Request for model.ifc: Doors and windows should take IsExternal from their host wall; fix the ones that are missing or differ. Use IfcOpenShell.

First a look at what the model holds.

```python
import ifcopenshell
import ifcopenshell.util.element

model = ifcopenshell.open("model.ifc")
print(model.schema)
seen = {}
for e in model.by_type("IfcDoor") + model.by_type("IfcWindow"):
    if not e.FillsVoids:
        continue
    host = e.FillsVoids[0].RelatingOpeningElement.VoidsElements[0].RelatingBuildingElement
    own = ifcopenshell.util.element.get_pset(e, f"Pset_{e.is_a()[3:].removesuffix('StandardCase')}Common", "IsExternal")
    wall = ifcopenshell.util.element.get_pset(host, "Pset_WallCommon", "IsExternal")
    seen[e.is_a(), own, wall] = seen.get((e.is_a(), own, wall), 0) + 1
for (cls, own, wall), count in sorted(seen.items(), key=str):
    print(count, cls, "IsExternal:", own, "| host wall:", wall)
```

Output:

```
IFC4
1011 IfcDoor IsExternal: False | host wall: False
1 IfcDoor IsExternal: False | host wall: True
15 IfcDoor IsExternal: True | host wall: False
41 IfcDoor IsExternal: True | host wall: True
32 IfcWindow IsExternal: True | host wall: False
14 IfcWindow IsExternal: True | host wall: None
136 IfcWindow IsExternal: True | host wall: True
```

```python
import ifcopenshell
import ifcopenshell.api.pset
import ifcopenshell.util.element

model = ifcopenshell.open("model.ifc")

count = 0
for ifc_class, pset_name in (("IfcDoor", "Pset_DoorCommon"), ("IfcWindow", "Pset_WindowCommon")):
    for e in model.by_type(ifc_class):
        if not e.FillsVoids:
            continue
        host = e.FillsVoids[0].RelatingOpeningElement.VoidsElements[0].RelatingBuildingElement
        external = ifcopenshell.util.element.get_pset(host, "Pset_WallCommon", "IsExternal")
        if external is None or ifcopenshell.util.element.get_pset(e, pset_name, "IsExternal") == external:
            continue
        pset = ifcopenshell.api.pset.add_pset(model, product=e, name=pset_name)
        ifcopenshell.api.pset.edit_pset(model, pset=pset, properties={"IsExternal": external})
        count += 1

print(count, "updated")

model.write("model_rev.ifc")
```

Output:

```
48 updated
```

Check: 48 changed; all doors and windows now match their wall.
